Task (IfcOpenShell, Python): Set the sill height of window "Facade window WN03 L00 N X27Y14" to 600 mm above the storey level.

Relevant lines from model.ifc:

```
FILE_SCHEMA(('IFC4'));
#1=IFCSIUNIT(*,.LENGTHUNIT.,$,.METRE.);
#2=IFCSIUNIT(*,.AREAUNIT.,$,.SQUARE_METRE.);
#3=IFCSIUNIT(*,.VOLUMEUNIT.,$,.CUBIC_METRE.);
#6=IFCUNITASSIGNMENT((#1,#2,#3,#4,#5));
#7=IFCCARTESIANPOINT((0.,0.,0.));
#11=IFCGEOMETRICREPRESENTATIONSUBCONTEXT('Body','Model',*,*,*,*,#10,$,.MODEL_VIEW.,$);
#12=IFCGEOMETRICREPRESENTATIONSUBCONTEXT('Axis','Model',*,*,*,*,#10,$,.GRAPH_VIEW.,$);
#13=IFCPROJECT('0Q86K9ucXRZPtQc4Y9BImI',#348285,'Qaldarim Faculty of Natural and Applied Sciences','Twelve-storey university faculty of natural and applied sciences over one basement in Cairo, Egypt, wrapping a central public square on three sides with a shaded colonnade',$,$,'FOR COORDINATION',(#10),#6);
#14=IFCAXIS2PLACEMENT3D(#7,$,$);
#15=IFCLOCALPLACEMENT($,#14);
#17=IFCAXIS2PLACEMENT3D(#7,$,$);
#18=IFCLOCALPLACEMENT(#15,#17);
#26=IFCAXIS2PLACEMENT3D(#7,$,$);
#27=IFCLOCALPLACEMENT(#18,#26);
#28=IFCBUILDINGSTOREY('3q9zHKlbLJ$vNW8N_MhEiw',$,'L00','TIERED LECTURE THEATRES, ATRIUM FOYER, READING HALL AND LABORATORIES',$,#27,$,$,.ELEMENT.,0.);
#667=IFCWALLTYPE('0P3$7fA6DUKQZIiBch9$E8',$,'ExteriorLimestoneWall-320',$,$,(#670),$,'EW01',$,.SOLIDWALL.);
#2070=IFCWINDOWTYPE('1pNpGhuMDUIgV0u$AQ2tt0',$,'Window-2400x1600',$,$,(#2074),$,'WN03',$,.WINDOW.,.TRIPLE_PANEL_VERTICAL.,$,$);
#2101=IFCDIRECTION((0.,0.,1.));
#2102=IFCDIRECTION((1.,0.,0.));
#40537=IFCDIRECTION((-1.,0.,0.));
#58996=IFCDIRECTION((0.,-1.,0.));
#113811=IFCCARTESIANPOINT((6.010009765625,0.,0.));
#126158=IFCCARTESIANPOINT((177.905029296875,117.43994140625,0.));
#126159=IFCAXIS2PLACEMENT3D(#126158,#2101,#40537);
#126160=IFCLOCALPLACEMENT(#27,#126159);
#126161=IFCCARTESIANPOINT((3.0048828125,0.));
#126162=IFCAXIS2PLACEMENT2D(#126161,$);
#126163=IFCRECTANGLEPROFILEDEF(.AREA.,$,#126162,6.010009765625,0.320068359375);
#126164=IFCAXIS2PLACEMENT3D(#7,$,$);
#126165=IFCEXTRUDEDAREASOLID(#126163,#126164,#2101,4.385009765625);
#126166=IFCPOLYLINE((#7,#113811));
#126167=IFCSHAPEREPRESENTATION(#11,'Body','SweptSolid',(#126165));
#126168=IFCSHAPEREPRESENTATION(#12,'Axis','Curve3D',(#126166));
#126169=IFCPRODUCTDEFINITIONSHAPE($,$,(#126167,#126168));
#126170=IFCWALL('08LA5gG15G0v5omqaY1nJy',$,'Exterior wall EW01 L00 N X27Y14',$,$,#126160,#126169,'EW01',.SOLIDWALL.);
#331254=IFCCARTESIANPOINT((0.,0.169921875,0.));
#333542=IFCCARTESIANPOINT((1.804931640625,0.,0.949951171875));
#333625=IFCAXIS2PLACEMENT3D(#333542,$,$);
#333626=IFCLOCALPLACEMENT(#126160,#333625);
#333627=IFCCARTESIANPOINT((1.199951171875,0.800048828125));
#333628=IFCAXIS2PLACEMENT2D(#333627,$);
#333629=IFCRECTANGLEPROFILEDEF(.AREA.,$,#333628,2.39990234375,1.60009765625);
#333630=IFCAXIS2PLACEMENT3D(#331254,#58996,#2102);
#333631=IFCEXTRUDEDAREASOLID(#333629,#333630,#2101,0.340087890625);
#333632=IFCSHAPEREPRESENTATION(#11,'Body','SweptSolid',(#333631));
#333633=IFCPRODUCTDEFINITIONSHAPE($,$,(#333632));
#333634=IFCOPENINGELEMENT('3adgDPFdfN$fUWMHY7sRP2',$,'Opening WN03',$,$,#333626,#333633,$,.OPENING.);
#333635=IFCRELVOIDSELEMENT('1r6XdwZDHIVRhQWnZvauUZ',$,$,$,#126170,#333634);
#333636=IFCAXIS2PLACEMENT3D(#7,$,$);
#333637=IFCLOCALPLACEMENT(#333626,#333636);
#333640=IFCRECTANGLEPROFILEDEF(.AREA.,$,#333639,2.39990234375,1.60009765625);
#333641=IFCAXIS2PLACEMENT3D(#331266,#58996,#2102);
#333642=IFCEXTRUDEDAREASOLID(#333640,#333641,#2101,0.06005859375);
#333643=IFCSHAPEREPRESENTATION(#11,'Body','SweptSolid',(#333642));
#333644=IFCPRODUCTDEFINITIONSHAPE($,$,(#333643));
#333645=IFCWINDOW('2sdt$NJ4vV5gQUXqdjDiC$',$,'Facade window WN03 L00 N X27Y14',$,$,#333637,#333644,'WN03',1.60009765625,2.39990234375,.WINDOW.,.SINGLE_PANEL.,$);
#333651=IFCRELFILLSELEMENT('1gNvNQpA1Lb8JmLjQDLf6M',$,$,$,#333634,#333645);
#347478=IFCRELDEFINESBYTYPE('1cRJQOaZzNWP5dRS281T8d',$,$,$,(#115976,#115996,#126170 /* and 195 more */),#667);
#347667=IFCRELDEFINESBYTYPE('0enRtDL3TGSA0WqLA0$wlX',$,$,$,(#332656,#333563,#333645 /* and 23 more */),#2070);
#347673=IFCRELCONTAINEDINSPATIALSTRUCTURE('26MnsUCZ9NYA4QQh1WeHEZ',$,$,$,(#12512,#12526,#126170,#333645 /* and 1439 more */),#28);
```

```python
import numpy as np
import ifcopenshell
import ifcopenshell.api.geometry
import ifcopenshell.geom
import ifcopenshell.util.element
import ifcopenshell.util.placement
import ifcopenshell.util.shape
import ifcopenshell.util.unit

model = ifcopenshell.open("model.ifc")
unit_scale = ifcopenshell.util.unit.calculate_unit_scale(model)

window = model.by_guid("2sdt$NJ4vV5gQUXqdjDiC$")
opening = window.FillsVoids[0].RelatingOpeningElement
storey = ifcopenshell.util.element.get_container(window, ifc_class="IfcBuildingStorey")
level = ifcopenshell.util.placement.get_local_placement(storey.ObjectPlacement)[2, 3]

# The opening's origin need not be at the sill, so measure its lowest point.
shape = ifcopenshell.geom.create_shape(ifcopenshell.geom.settings(), opening)
bottom = ifcopenshell.util.shape.get_shape_bottom_elevation(shape, shape.geometry) / unit_scale
dz = level + 0.6 / unit_scale - bottom

shift = np.array([0.0, 0.0, dz])
# The window is placed relative to its opening, so it follows when the opening moves.
matrix = ifcopenshell.util.placement.get_local_placement(opening.ObjectPlacement)
matrix[:3, 3] += shift
ifcopenshell.api.geometry.edit_object_placement(
    model, product=opening, matrix=matrix, is_si=False, should_transform_children=True
)

print(f"moved by {dz * unit_scale:+.3f} m")

model.write("model_rev.ifc")
```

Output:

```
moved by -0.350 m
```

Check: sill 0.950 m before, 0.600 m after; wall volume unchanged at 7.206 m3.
